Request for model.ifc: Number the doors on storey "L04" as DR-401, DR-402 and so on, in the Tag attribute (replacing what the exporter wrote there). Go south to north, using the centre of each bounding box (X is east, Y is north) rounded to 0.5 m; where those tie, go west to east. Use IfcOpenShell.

First a look at what the model holds.

```python
import ifcopenshell
import ifcopenshell.util.element
import ifcopenshell.util.placement

model = ifcopenshell.open("model.ifc")
print(model.schema)
storey = next(s for s in model.by_type("IfcBuildingStorey") if s.Name == "L04")
doors = [e for e in ifcopenshell.util.element.get_decomposition(storey) if e.is_a("IfcDoor")]
for e in sorted(doors, key=lambda e: e.id()):
    origin = ifcopenshell.util.placement.get_local_placement(e.ObjectPlacement)[:3, 3]
    print(e.id(), e.Tag, e.Name, origin.round(2) + 0.0, sep=" | ")
```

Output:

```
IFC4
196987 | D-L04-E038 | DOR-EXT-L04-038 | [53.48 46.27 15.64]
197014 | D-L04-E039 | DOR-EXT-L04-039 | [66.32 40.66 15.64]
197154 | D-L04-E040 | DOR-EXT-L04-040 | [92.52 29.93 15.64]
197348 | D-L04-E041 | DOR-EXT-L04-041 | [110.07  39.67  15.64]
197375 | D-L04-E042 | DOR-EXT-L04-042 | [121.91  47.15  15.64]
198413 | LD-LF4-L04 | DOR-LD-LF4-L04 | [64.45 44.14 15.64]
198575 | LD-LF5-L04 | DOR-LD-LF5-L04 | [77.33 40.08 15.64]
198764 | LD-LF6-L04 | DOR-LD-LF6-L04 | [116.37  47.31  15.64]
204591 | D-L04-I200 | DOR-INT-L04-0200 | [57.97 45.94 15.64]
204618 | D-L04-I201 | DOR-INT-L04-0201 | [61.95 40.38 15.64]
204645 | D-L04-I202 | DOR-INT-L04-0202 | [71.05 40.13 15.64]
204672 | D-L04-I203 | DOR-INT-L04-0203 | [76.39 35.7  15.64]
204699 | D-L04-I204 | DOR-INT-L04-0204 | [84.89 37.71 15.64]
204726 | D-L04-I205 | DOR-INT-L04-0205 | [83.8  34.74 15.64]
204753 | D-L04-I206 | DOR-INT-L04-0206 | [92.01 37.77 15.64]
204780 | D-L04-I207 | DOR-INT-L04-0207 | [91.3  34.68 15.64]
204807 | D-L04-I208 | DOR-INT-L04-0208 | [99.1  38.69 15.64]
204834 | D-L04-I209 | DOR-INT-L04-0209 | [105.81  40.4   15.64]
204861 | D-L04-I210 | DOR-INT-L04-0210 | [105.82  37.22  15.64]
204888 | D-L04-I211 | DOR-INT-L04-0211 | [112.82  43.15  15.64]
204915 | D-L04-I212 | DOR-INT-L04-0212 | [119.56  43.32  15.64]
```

```python
import ifcopenshell
import ifcopenshell.geom
import ifcopenshell.util.element
import ifcopenshell.util.shape

model = ifcopenshell.open("model.ifc")
settings = ifcopenshell.geom.settings()
settings.set("use-world-coords", True)


def centre(element):
    shape = ifcopenshell.geom.create_shape(settings, element)
    return ifcopenshell.util.shape.get_bbox_centroid(shape.geometry)


storey = next(s for s in model.by_type("IfcBuildingStorey") if s.Name == "L04")
doors = [e for e in ifcopenshell.util.element.get_decomposition(storey) if e.is_a("IfcDoor")]

# Insertion points can sit at a corner or the storey origin, so sort by the geometry (in metres).
centres = {e: centre(e) for e in doors}
doors.sort(key=lambda e: (round(centres[e][1] / 0.5), centres[e][0]))

for i, e in enumerate(doors, start=1):
    number = f"DR-4{i:02d}"
    e.Tag = number
    print(e.id(), number)

model.write("model-out.ifc")
```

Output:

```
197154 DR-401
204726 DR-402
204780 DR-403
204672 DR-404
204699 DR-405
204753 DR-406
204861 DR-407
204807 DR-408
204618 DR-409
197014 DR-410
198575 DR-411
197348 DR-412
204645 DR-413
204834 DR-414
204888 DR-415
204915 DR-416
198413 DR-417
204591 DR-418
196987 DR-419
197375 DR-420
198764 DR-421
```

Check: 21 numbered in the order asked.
